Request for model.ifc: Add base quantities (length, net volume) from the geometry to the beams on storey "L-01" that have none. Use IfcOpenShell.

First a look at what the model holds.

```python
import ifcopenshell
import ifcopenshell.util.element
import ifcopenshell.util.unit

model = ifcopenshell.open("model.ifc")
print(model.schema)
for unit_type in ("LENGTHUNIT", "AREAUNIT", "VOLUMEUNIT"):
    print(unit_type, ifcopenshell.util.unit.calculate_unit_scale(model, unit_type))
storey = next(s for s in model.by_type("IfcBuildingStorey") if s.Name == "L-01")
beams = [e for e in ifcopenshell.util.element.get_decomposition(storey) if e.is_a("IfcBeam")]
for e in sorted(beams, key=lambda e: e.id()):
    print(e.id(), e.is_a(), e.Name, list(ifcopenshell.util.element.get_psets(e, qtos_only=True)), sep=" | ")
```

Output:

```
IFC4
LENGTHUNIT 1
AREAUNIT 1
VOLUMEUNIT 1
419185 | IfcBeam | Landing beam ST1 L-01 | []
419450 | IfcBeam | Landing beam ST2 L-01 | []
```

```python
import ifcopenshell
import ifcopenshell.api.pset
import ifcopenshell.geom
import ifcopenshell.util.element
import ifcopenshell.util.shape
import ifcopenshell.util.unit

model = ifcopenshell.open("model.ifc")
unit_scale = ifcopenshell.util.unit.calculate_unit_scale(model)
volume_scale = ifcopenshell.util.unit.calculate_unit_scale(model, "VOLUMEUNIT")
settings = ifcopenshell.geom.settings()

storey = next(s for s in model.by_type("IfcBuildingStorey") if s.Name == "L-01")
beams = [e for e in ifcopenshell.util.element.get_decomposition(storey) if e.is_a("IfcBeam")]

for e in sorted(beams, key=lambda e: e.id()):
    if ifcopenshell.util.element.get_psets(e, qtos_only=True, should_inherit=False):
        continue
    # Geometry comes back in metres, in the element's own axes.
    shape = ifcopenshell.geom.create_shape(settings, e)
    values = {
        "Length": ifcopenshell.util.shape.get_max_xyz(shape.geometry) / unit_scale,
        "NetVolume": ifcopenshell.util.shape.get_volume(shape.geometry) / volume_scale,
    }
    qto = ifcopenshell.api.pset.add_qto(model, product=e, name="Qto_BeamBaseQuantities")
    ifcopenshell.api.pset.edit_qto(model, qto=qto, properties=values)
    print(e.id(), {k: round(v, 3) for k, v in values.items()})

model.write("model_updated.ifc")
```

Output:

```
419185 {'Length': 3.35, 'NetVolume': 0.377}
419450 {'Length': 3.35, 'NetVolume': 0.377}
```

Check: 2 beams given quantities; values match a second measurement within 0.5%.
